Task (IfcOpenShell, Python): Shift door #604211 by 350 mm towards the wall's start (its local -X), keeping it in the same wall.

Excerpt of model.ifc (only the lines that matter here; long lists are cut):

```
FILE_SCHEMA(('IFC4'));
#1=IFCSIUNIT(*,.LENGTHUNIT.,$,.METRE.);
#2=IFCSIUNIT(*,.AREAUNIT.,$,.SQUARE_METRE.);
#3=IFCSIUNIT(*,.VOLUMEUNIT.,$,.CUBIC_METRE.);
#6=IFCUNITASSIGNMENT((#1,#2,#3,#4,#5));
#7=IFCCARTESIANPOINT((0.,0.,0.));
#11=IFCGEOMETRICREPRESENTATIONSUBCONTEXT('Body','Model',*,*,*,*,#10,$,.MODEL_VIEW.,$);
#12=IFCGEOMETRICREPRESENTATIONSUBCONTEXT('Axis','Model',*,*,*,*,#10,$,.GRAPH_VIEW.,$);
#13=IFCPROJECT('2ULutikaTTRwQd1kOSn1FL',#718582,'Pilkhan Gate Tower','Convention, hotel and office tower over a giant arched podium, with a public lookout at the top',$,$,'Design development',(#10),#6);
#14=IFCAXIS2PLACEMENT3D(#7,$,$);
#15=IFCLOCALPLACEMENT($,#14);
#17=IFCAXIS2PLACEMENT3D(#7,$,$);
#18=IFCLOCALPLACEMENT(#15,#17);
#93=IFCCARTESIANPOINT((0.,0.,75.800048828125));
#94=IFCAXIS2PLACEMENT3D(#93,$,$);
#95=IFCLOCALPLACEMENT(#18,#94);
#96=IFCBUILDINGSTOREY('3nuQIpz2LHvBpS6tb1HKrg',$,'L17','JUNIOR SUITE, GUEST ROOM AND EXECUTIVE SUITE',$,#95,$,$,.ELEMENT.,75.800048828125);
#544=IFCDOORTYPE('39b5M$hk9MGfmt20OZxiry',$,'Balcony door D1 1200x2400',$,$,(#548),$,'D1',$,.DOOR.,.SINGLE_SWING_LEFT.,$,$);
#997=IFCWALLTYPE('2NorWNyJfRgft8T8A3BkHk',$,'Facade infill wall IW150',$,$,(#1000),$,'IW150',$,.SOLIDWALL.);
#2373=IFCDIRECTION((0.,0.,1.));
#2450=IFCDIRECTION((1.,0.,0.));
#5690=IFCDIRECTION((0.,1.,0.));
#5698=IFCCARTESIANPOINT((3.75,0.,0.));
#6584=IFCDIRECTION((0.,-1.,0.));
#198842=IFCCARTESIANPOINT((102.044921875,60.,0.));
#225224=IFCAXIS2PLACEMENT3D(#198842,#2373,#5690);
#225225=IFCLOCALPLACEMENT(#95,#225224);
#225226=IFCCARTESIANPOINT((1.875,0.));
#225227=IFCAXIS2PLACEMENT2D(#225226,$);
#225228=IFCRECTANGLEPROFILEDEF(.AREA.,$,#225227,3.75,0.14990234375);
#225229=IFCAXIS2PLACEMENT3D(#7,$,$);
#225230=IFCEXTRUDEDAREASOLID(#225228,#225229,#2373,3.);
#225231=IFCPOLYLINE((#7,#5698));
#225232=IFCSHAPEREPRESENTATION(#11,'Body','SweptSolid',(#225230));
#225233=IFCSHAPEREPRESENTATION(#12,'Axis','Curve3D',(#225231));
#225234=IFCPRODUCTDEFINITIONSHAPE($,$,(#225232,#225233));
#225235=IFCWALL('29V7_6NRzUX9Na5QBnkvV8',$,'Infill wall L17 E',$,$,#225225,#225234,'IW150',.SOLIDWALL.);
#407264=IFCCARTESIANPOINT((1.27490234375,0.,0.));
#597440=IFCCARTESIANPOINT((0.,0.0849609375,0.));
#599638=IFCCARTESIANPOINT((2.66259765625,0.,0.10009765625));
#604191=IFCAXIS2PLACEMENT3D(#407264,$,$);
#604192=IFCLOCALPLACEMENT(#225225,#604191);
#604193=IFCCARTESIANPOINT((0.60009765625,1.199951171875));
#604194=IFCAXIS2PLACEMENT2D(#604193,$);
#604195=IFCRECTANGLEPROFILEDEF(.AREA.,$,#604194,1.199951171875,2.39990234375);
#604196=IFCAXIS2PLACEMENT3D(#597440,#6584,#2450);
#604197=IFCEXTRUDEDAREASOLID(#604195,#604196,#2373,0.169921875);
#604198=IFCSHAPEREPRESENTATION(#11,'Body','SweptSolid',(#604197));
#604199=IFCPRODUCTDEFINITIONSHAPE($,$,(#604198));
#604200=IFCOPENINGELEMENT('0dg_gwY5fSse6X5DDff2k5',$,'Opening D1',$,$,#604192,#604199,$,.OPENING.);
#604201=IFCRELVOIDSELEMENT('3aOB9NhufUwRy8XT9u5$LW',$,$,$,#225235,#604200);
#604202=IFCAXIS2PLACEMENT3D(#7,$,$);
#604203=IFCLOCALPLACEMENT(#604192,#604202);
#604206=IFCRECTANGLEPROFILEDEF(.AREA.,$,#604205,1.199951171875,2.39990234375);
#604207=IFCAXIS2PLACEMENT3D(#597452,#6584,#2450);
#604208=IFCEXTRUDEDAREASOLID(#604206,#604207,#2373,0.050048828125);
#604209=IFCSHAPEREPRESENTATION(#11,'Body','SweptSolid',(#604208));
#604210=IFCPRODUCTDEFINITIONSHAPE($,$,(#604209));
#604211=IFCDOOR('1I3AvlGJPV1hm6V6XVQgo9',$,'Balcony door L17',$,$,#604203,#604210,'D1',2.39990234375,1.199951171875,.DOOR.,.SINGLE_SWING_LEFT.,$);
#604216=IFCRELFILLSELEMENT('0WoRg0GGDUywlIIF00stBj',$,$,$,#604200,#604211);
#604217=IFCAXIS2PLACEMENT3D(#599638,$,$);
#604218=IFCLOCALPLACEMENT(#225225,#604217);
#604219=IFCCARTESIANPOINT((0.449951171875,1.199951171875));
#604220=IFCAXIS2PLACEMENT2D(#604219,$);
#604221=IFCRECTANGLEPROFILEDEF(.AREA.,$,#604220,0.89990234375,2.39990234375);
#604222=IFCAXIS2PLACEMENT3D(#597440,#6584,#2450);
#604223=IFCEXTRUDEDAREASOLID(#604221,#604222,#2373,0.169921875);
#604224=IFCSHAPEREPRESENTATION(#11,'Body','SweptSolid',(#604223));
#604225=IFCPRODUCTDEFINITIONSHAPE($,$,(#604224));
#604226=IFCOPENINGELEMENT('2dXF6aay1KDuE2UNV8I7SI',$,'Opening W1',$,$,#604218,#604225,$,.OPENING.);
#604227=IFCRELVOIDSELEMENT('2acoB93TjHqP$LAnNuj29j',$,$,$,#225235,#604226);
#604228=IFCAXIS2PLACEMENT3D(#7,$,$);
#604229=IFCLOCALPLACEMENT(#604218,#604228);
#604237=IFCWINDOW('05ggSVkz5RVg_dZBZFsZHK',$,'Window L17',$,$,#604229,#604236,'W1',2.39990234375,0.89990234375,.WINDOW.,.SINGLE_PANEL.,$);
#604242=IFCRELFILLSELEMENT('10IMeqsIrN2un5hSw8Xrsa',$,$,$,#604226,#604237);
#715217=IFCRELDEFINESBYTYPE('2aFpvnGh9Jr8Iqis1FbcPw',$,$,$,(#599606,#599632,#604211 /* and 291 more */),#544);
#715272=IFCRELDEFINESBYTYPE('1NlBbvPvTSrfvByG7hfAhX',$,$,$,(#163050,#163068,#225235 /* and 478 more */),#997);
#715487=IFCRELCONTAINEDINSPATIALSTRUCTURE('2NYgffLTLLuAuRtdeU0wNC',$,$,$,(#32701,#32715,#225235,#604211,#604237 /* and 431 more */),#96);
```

```python
import ifcopenshell
import ifcopenshell.api.geometry
import ifcopenshell.util.placement

model = ifcopenshell.open("model.ifc")

door = model.by_guid("1I3AvlGJPV1hm6V6XVQgo9")
opening = door.FillsVoids[0].RelatingOpeningElement
wall = opening.VoidsElements[0].RelatingBuildingElement

wall_matrix = ifcopenshell.util.placement.get_local_placement(wall.ObjectPlacement)
shift = wall_matrix[:3, 0] * -0.35
before = ifcopenshell.util.placement.get_local_placement(door.ObjectPlacement)[:3, 3].copy()

# The door is placed relative to its opening, so it follows when the opening moves.
matrix = ifcopenshell.util.placement.get_local_placement(opening.ObjectPlacement)
matrix[:3, 3] += shift
ifcopenshell.api.geometry.edit_object_placement(
    model, product=opening, matrix=matrix, is_si=False, should_transform_children=True
)

after = ifcopenshell.util.placement.get_local_placement(door.ObjectPlacement)[:3, 3]
print("door moved by", (after - before).round(3) + 0.0)

model.write("model_edited.ifc")
```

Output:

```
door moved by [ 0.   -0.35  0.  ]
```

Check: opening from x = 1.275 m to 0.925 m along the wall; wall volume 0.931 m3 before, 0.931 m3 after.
